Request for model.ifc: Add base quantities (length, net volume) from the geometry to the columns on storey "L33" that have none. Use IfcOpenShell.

First a look at what the model holds.

```python
import ifcopenshell
import ifcopenshell.util.element
import ifcopenshell.util.unit

model = ifcopenshell.open("model.ifc")
print(model.schema)
for unit_type in ("LENGTHUNIT", "AREAUNIT", "VOLUMEUNIT"):
    print(unit_type, ifcopenshell.util.unit.calculate_unit_scale(model, unit_type))
storey = next(s for s in model.by_type("IfcBuildingStorey") if s.Name == "L33")
columns = [e for e in ifcopenshell.util.element.get_decomposition(storey) if e.is_a("IfcColumn")]
for e in sorted(columns, key=lambda e: e.id()):
    print(e.id(), e.is_a(), e.Name, list(ifcopenshell.util.element.get_psets(e, qtos_only=True)), sep=" | ")
```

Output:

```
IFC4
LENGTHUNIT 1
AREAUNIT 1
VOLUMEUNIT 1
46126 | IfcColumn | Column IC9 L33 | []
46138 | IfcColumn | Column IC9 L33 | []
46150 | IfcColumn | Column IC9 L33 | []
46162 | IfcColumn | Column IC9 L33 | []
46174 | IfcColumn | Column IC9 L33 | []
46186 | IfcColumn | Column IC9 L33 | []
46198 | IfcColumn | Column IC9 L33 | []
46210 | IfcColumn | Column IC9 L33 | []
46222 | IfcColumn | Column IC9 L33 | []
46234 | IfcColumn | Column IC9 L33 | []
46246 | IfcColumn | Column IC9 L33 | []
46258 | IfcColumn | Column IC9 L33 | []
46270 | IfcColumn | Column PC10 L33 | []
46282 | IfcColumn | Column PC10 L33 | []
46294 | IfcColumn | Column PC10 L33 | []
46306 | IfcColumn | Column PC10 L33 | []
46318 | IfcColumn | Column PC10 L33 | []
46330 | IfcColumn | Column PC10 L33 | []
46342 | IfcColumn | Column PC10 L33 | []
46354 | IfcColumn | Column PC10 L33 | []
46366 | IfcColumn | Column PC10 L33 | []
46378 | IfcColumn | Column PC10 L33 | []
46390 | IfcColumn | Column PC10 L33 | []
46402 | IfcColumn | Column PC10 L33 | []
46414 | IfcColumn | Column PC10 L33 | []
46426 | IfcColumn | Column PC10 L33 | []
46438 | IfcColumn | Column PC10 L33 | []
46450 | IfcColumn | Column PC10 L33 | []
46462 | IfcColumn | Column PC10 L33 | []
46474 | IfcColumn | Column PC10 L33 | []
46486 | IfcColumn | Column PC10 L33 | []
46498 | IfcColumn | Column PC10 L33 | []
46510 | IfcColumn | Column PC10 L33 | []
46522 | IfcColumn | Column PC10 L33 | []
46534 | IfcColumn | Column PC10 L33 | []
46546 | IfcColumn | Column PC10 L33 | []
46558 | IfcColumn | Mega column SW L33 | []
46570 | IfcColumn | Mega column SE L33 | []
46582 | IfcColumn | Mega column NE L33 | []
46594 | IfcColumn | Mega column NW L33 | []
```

```python
import ifcopenshell
import ifcopenshell.api.pset
import ifcopenshell.geom
import ifcopenshell.util.element
import ifcopenshell.util.shape
import ifcopenshell.util.unit

model = ifcopenshell.open("model.ifc")
unit_scale = ifcopenshell.util.unit.calculate_unit_scale(model)
volume_scale = ifcopenshell.util.unit.calculate_unit_scale(model, "VOLUMEUNIT")
settings = ifcopenshell.geom.settings()

storey = next(s for s in model.by_type("IfcBuildingStorey") if s.Name == "L33")
columns = [e for e in ifcopenshell.util.element.get_decomposition(storey) if e.is_a("IfcColumn")]

for e in sorted(columns, key=lambda e: e.id()):
    if ifcopenshell.util.element.get_psets(e, qtos_only=True, should_inherit=False):
        continue
    # Geometry comes back in metres, in the element's own axes.
    shape = ifcopenshell.geom.create_shape(settings, e)
    values = {
        "Length": ifcopenshell.util.shape.get_z(shape.geometry) / unit_scale,
        "NetVolume": ifcopenshell.util.shape.get_volume(shape.geometry) / volume_scale,
    }
    qto = ifcopenshell.api.pset.add_qto(model, product=e, name="Qto_ColumnBaseQuantities")
    ifcopenshell.api.pset.edit_qto(model, qto=qto, properties=values)
    print(e.id(), {k: round(v, 3) for k, v in values.items()})

model.write("model_edited.ifc")
```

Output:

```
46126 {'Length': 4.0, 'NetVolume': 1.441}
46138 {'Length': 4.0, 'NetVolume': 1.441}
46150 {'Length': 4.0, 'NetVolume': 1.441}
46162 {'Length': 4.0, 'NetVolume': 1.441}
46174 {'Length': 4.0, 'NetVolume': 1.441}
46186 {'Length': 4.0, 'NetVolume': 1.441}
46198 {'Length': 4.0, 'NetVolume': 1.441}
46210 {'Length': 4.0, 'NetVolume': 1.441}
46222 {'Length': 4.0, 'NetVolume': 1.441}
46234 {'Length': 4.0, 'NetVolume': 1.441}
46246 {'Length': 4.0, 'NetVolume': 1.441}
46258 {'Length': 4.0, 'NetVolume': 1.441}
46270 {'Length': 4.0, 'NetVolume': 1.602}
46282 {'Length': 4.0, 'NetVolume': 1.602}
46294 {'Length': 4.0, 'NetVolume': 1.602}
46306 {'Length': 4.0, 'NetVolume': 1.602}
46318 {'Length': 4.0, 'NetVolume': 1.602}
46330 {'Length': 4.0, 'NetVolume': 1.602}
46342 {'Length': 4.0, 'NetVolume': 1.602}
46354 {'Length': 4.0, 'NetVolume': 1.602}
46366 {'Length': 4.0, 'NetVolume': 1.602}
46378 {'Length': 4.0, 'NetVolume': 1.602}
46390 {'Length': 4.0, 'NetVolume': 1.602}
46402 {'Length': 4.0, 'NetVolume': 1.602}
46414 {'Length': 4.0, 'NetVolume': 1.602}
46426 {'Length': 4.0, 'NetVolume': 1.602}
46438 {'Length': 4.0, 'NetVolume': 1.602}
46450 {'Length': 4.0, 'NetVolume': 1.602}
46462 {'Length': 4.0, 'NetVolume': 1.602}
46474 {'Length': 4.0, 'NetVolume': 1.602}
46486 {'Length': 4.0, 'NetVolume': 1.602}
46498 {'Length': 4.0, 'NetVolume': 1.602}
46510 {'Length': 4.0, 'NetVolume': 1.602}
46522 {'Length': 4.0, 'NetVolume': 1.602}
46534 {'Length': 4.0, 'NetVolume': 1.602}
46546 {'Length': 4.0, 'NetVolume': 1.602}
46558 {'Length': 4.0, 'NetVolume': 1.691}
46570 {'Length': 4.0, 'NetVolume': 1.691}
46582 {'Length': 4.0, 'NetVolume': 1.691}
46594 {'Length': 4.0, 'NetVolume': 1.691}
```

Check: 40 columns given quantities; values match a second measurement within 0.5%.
